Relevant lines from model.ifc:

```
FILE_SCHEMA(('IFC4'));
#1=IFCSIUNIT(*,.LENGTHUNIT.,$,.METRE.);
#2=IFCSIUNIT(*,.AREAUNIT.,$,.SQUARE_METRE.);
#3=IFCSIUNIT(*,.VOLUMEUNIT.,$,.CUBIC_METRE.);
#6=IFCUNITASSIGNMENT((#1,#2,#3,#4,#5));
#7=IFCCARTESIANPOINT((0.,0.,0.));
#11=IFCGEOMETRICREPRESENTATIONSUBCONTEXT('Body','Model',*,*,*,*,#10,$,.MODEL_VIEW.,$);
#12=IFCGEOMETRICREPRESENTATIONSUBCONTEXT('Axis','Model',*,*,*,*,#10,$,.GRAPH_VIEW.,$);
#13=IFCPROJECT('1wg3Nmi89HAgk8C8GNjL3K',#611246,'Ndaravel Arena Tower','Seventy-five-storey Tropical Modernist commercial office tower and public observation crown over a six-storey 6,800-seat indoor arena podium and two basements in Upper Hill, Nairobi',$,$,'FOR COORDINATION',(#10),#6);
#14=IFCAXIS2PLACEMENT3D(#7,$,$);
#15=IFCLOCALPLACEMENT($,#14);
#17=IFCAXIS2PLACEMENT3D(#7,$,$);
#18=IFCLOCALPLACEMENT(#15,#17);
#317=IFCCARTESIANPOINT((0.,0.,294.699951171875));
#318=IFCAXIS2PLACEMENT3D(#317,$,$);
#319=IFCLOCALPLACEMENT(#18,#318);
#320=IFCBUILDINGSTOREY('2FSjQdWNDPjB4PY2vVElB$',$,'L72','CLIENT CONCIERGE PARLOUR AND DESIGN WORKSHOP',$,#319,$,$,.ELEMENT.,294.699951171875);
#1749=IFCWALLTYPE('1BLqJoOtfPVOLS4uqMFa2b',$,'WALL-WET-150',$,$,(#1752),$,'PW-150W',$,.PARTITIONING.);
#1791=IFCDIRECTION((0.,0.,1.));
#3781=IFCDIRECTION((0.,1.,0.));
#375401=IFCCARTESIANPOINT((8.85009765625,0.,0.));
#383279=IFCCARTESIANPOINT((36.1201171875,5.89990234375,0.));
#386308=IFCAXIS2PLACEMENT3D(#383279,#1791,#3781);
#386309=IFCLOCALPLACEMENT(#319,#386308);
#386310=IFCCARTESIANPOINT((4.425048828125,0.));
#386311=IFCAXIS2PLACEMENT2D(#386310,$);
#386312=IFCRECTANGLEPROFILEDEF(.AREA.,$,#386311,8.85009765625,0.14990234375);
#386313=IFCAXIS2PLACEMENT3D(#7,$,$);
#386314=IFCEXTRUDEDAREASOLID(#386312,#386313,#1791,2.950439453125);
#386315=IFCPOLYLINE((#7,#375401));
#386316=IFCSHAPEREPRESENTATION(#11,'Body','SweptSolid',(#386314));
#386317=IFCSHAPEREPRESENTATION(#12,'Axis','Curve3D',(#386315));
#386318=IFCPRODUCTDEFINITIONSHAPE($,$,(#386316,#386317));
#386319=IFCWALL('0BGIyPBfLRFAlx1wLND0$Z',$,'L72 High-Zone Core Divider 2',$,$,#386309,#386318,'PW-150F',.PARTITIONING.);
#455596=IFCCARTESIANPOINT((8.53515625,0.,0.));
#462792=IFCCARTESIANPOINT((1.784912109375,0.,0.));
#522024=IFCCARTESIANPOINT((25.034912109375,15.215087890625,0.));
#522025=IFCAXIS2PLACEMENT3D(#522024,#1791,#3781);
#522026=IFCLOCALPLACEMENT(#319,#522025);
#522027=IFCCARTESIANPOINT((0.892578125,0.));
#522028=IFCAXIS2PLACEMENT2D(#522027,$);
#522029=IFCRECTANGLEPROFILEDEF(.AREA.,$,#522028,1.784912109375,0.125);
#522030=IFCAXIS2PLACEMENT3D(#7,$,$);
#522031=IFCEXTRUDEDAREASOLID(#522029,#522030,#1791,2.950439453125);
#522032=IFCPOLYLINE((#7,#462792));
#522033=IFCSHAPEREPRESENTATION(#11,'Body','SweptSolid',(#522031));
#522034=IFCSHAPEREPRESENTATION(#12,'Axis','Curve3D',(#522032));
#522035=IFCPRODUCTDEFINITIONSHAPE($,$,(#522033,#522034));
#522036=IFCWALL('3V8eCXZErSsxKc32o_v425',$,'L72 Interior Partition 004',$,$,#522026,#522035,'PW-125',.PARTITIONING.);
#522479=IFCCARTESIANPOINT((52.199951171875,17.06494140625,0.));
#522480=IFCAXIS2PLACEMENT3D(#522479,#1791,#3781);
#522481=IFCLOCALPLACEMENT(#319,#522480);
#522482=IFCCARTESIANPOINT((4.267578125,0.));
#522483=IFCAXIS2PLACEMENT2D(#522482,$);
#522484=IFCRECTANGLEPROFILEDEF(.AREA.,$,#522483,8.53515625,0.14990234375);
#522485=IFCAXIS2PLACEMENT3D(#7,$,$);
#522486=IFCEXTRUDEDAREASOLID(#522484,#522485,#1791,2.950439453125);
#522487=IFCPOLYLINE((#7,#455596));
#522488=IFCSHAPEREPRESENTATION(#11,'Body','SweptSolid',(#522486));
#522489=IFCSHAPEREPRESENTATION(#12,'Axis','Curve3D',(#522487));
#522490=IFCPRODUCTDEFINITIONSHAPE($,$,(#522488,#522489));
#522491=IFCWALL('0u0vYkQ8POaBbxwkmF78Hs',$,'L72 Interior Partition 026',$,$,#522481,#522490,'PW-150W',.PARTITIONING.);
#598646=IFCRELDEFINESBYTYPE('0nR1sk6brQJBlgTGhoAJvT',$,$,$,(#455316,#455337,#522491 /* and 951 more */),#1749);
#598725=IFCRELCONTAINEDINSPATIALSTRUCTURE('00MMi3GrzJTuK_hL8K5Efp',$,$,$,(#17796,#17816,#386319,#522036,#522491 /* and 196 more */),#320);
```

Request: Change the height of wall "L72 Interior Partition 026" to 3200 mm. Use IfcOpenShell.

```python
import ifcopenshell
import ifcopenshell.geom
import ifcopenshell.util.representation
import ifcopenshell.util.shape
import ifcopenshell.util.unit

model = ifcopenshell.open("model.ifc")
unit_scale = ifcopenshell.util.unit.calculate_unit_scale(model)
settings = ifcopenshell.geom.settings()


def volume(element):
    """Net volume in cubic metres, openings subtracted."""
    shape = ifcopenshell.geom.create_shape(settings, element)
    return ifcopenshell.util.shape.get_volume(shape.geometry)


wall = model.by_guid("0u0vYkQ8POaBbxwkmF78Hs")
before = volume(wall)

body = ifcopenshell.util.representation.get_representation(wall, "Model", "Body")
solid = body.Items[0]
old_height = solid.Depth
solid.Depth = 3.2 / unit_scale
after = volume(wall)

print(f"height {old_height:g} -> {solid.Depth:g}, volume {before:.3f} -> {after:.3f} m3")

model.write("model_edited.ifc")
```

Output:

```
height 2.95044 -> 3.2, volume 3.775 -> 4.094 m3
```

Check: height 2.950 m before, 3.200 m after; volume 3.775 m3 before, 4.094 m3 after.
